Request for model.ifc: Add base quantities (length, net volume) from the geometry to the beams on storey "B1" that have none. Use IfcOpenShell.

First a look at what the model holds.

```python
import ifcopenshell
import ifcopenshell.util.element
import ifcopenshell.util.unit

model = ifcopenshell.open("model.ifc")
print(model.schema)
for unit_type in ("LENGTHUNIT", "AREAUNIT", "VOLUMEUNIT"):
    print(unit_type, ifcopenshell.util.unit.calculate_unit_scale(model, unit_type))
storey = next(s for s in model.by_type("IfcBuildingStorey") if s.Name == "B1")
beams = [e for e in ifcopenshell.util.element.get_decomposition(storey) if e.is_a("IfcBeam")]
for e in sorted(beams, key=lambda e: e.id()):
    print(e.id(), e.is_a(), e.Name, list(ifcopenshell.util.element.get_psets(e, qtos_only=True)), sep=" | ")
```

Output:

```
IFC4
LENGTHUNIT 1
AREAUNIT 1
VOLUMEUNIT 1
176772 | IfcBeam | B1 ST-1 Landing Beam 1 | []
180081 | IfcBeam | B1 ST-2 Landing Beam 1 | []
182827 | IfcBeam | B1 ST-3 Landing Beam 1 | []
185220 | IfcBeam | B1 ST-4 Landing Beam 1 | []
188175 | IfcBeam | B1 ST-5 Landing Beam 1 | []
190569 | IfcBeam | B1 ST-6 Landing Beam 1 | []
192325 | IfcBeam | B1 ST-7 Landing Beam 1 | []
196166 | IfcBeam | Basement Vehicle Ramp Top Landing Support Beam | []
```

```python
import ifcopenshell
import ifcopenshell.api.pset
import ifcopenshell.geom
import ifcopenshell.util.element
import ifcopenshell.util.shape
import ifcopenshell.util.unit

model = ifcopenshell.open("model.ifc")
unit_scale = ifcopenshell.util.unit.calculate_unit_scale(model)
volume_scale = ifcopenshell.util.unit.calculate_unit_scale(model, "VOLUMEUNIT")
settings = ifcopenshell.geom.settings()

storey = next(s for s in model.by_type("IfcBuildingStorey") if s.Name == "B1")
beams = [e for e in ifcopenshell.util.element.get_decomposition(storey) if e.is_a("IfcBeam")]

for e in sorted(beams, key=lambda e: e.id()):
    if ifcopenshell.util.element.get_psets(e, qtos_only=True, should_inherit=False):
        continue
    # Geometry comes back in metres, in the element's own axes.
    shape = ifcopenshell.geom.create_shape(settings, e)
    values = {
        "Length": ifcopenshell.util.shape.get_max_xyz(shape.geometry) / unit_scale,
        "NetVolume": ifcopenshell.util.shape.get_volume(shape.geometry) / volume_scale,
    }
    qto = ifcopenshell.api.pset.add_qto(model, product=e, name="Qto_BeamBaseQuantities")
    ifcopenshell.api.pset.edit_qto(model, qto=qto, properties=values)
    print(e.id(), {k: round(v, 3) for k, v in values.items()})

model.write("model-out.ifc")
```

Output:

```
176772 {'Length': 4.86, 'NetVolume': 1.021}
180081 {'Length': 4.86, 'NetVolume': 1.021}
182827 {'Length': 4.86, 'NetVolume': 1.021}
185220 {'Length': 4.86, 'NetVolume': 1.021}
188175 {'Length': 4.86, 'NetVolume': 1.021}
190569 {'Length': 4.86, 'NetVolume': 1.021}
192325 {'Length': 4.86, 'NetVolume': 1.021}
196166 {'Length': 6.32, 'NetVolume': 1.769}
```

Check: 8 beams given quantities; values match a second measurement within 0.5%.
